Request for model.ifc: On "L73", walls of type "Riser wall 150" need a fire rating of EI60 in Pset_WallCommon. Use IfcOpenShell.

First a look at what the model holds.

```python
import ifcopenshell
import ifcopenshell.util.element

model = ifcopenshell.open("model.ifc")
print(model.schema)
storey = next(s for s in model.by_type("IfcBuildingStorey") if s.Name == "L73")
walls = [e for e in ifcopenshell.util.element.get_decomposition(storey) if e.is_a("IfcWall")]
seen = {}
for e in walls:
    element_type = ifcopenshell.util.element.get_type(e)
    key = (element_type.Name if element_type != e and element_type else None, ifcopenshell.util.element.get_pset(e, "Pset_WallCommon", "FireRating"))
    seen[key] = seen.get(key, 0) + 1
for (name, value), count in sorted(seen.items(), key=str):
    print(count, "x", name, "|", value)
```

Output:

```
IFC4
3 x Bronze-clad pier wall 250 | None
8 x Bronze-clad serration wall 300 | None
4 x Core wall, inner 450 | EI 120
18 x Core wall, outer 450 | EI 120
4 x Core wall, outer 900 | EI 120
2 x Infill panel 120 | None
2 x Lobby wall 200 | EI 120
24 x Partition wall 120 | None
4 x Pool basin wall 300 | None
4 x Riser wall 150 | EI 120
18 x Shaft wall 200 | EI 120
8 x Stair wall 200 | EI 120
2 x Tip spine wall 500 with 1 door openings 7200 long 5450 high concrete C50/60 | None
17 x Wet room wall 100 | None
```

```python
import ifcopenshell
import ifcopenshell.api.pset
import ifcopenshell.util.element

model = ifcopenshell.open("model.ifc")

storey = next(s for s in model.by_type("IfcBuildingStorey") if s.Name == "L73")
walls = [e for e in ifcopenshell.util.element.get_decomposition(storey) if e.is_a("IfcWall")]

count = 0
for e in walls:
    element_type = ifcopenshell.util.element.get_type(e)
    if element_type in (None, e) or element_type.Name != "Riser wall 150":
        continue
    found = ifcopenshell.util.element.get_pset(e, "Pset_WallCommon", should_inherit=False)
    if found:
        pset = model.by_id(found["id"])
        if len(ifcopenshell.util.element.get_elements_by_pset(pset)) > 1:
            pset = ifcopenshell.api.pset.unshare_pset(model, products=[e], pset=pset)[0]
    else:
        pset = ifcopenshell.api.pset.add_pset(model, product=e, name="Pset_WallCommon")
    ifcopenshell.api.pset.edit_pset(model, pset=pset, properties={"FireRating": "EI60"})
    count += 1

print(count, "walls updated")

model.write("model_updated.ifc")
```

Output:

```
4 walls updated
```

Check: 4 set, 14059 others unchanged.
